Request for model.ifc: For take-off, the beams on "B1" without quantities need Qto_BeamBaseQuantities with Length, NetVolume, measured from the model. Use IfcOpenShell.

First a look at what the model holds.

```python
import ifcopenshell
import ifcopenshell.util.element
import ifcopenshell.util.unit

model = ifcopenshell.open("model.ifc")
print(model.schema)
for unit_type in ("LENGTHUNIT", "AREAUNIT", "VOLUMEUNIT"):
    print(unit_type, ifcopenshell.util.unit.calculate_unit_scale(model, unit_type))
storey = next(s for s in model.by_type("IfcBuildingStorey") if s.Name == "B1")
beams = [e for e in ifcopenshell.util.element.get_decomposition(storey) if e.is_a("IfcBeam")]
for e in sorted(beams, key=lambda e: e.id()):
    print(e.id(), e.is_a(), e.Name, list(ifcopenshell.util.element.get_psets(e, qtos_only=True)), sep=" | ")
```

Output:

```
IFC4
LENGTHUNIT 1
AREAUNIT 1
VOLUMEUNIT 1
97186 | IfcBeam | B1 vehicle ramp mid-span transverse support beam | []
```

```python
import ifcopenshell
import ifcopenshell.api.pset
import ifcopenshell.geom
import ifcopenshell.util.element
import ifcopenshell.util.shape
import ifcopenshell.util.unit

model = ifcopenshell.open("model.ifc")
unit_scale = ifcopenshell.util.unit.calculate_unit_scale(model)
volume_scale = ifcopenshell.util.unit.calculate_unit_scale(model, "VOLUMEUNIT")
settings = ifcopenshell.geom.settings()

storey = next(s for s in model.by_type("IfcBuildingStorey") if s.Name == "B1")
beams = [e for e in ifcopenshell.util.element.get_decomposition(storey) if e.is_a("IfcBeam")]

for e in sorted(beams, key=lambda e: e.id()):
    if ifcopenshell.util.element.get_psets(e, qtos_only=True, should_inherit=False):
        continue
    # Geometry comes back in metres, in the element's own axes.
    shape = ifcopenshell.geom.create_shape(settings, e)
    values = {
        "Length": ifcopenshell.util.shape.get_max_xyz(shape.geometry) / unit_scale,
        "NetVolume": ifcopenshell.util.shape.get_volume(shape.geometry) / volume_scale,
    }
    qto = ifcopenshell.api.pset.add_qto(model, product=e, name="Qto_BeamBaseQuantities")
    ifcopenshell.api.pset.edit_qto(model, qto=qto, properties=values)
    print(e.id(), {k: round(v, 3) for k, v in values.items()})

model.write("model_updated.ifc")
```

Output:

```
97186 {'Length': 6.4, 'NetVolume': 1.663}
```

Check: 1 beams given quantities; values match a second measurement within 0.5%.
